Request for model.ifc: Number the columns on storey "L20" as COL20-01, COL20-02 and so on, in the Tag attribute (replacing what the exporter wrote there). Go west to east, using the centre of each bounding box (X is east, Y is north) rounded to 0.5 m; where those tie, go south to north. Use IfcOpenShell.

First a look at what the model holds.

```python
import ifcopenshell
import ifcopenshell.util.element
import ifcopenshell.util.placement

model = ifcopenshell.open("model.ifc")
print(model.schema)
storey = next(s for s in model.by_type("IfcBuildingStorey") if s.Name == "L20")
columns = [e for e in ifcopenshell.util.element.get_decomposition(storey) if e.is_a("IfcColumn")]
for e in sorted(columns, key=lambda e: e.id()):
    origin = ifcopenshell.util.placement.get_local_placement(e.ObjectPlacement)[:3, 3]
    print(e.id(), e.Tag, e.Name, origin.round(2) + 0.0, sep=" | ")
```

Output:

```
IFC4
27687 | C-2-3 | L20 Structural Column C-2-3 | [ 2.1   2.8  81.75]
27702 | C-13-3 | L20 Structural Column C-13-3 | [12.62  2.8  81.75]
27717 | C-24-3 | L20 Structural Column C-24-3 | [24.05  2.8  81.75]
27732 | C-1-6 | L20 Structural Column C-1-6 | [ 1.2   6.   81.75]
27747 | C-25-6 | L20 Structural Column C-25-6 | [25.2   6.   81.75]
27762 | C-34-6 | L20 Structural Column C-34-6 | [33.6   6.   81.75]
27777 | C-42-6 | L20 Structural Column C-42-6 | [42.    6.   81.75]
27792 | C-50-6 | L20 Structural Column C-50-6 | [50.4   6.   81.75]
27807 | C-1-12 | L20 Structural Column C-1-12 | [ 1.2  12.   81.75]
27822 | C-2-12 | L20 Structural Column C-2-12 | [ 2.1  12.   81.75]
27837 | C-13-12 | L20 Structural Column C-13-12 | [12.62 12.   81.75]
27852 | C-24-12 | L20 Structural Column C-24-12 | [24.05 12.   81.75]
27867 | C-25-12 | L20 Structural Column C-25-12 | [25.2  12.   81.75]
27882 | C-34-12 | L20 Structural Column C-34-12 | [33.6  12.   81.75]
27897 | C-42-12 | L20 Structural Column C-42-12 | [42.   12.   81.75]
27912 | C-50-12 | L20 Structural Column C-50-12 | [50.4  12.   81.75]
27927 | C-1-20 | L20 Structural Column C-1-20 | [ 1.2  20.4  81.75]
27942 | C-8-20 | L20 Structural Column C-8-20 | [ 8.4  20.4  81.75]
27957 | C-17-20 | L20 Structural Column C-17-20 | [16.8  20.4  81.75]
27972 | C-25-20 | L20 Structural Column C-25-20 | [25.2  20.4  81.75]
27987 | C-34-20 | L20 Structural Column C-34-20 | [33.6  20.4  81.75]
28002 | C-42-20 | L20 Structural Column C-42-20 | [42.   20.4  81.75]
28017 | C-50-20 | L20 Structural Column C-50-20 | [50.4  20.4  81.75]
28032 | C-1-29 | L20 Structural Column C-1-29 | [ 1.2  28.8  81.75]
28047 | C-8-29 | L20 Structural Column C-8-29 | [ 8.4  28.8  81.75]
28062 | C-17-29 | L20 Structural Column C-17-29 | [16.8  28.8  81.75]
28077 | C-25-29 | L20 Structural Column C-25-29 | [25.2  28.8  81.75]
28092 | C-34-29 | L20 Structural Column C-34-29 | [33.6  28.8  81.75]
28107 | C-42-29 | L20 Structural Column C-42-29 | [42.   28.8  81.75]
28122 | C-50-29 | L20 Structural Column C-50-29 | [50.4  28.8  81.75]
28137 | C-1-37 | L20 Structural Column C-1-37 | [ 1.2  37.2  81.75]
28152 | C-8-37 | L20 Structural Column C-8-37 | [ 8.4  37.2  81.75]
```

```python
import ifcopenshell
import ifcopenshell.geom
import ifcopenshell.util.element
import ifcopenshell.util.shape

model = ifcopenshell.open("model.ifc")
settings = ifcopenshell.geom.settings()
settings.set("use-world-coords", True)


def centre(element):
    shape = ifcopenshell.geom.create_shape(settings, element)
    return ifcopenshell.util.shape.get_bbox_centroid(shape.geometry)


storey = next(s for s in model.by_type("IfcBuildingStorey") if s.Name == "L20")
columns = [e for e in ifcopenshell.util.element.get_decomposition(storey) if e.is_a("IfcColumn")]

# Insertion points can sit at a corner or the storey origin, so sort by the geometry (in metres).
centres = {e: centre(e) for e in columns}
columns.sort(key=lambda e: (round(centres[e][0] / 0.5), centres[e][1]))

for i, e in enumerate(columns, start=1):
    number = f"COL20-{i:02d}"
    e.Tag = number
    print(e.id(), number)

model.write("model_v2.ifc")
```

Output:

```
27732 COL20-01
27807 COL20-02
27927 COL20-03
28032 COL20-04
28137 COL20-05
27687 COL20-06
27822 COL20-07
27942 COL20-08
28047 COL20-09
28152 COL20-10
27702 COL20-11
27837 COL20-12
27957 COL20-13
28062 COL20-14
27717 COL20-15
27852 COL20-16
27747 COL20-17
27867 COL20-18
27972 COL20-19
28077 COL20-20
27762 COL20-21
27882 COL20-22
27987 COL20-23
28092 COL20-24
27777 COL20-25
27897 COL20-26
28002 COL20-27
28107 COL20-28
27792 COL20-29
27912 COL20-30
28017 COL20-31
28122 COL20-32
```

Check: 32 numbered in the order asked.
